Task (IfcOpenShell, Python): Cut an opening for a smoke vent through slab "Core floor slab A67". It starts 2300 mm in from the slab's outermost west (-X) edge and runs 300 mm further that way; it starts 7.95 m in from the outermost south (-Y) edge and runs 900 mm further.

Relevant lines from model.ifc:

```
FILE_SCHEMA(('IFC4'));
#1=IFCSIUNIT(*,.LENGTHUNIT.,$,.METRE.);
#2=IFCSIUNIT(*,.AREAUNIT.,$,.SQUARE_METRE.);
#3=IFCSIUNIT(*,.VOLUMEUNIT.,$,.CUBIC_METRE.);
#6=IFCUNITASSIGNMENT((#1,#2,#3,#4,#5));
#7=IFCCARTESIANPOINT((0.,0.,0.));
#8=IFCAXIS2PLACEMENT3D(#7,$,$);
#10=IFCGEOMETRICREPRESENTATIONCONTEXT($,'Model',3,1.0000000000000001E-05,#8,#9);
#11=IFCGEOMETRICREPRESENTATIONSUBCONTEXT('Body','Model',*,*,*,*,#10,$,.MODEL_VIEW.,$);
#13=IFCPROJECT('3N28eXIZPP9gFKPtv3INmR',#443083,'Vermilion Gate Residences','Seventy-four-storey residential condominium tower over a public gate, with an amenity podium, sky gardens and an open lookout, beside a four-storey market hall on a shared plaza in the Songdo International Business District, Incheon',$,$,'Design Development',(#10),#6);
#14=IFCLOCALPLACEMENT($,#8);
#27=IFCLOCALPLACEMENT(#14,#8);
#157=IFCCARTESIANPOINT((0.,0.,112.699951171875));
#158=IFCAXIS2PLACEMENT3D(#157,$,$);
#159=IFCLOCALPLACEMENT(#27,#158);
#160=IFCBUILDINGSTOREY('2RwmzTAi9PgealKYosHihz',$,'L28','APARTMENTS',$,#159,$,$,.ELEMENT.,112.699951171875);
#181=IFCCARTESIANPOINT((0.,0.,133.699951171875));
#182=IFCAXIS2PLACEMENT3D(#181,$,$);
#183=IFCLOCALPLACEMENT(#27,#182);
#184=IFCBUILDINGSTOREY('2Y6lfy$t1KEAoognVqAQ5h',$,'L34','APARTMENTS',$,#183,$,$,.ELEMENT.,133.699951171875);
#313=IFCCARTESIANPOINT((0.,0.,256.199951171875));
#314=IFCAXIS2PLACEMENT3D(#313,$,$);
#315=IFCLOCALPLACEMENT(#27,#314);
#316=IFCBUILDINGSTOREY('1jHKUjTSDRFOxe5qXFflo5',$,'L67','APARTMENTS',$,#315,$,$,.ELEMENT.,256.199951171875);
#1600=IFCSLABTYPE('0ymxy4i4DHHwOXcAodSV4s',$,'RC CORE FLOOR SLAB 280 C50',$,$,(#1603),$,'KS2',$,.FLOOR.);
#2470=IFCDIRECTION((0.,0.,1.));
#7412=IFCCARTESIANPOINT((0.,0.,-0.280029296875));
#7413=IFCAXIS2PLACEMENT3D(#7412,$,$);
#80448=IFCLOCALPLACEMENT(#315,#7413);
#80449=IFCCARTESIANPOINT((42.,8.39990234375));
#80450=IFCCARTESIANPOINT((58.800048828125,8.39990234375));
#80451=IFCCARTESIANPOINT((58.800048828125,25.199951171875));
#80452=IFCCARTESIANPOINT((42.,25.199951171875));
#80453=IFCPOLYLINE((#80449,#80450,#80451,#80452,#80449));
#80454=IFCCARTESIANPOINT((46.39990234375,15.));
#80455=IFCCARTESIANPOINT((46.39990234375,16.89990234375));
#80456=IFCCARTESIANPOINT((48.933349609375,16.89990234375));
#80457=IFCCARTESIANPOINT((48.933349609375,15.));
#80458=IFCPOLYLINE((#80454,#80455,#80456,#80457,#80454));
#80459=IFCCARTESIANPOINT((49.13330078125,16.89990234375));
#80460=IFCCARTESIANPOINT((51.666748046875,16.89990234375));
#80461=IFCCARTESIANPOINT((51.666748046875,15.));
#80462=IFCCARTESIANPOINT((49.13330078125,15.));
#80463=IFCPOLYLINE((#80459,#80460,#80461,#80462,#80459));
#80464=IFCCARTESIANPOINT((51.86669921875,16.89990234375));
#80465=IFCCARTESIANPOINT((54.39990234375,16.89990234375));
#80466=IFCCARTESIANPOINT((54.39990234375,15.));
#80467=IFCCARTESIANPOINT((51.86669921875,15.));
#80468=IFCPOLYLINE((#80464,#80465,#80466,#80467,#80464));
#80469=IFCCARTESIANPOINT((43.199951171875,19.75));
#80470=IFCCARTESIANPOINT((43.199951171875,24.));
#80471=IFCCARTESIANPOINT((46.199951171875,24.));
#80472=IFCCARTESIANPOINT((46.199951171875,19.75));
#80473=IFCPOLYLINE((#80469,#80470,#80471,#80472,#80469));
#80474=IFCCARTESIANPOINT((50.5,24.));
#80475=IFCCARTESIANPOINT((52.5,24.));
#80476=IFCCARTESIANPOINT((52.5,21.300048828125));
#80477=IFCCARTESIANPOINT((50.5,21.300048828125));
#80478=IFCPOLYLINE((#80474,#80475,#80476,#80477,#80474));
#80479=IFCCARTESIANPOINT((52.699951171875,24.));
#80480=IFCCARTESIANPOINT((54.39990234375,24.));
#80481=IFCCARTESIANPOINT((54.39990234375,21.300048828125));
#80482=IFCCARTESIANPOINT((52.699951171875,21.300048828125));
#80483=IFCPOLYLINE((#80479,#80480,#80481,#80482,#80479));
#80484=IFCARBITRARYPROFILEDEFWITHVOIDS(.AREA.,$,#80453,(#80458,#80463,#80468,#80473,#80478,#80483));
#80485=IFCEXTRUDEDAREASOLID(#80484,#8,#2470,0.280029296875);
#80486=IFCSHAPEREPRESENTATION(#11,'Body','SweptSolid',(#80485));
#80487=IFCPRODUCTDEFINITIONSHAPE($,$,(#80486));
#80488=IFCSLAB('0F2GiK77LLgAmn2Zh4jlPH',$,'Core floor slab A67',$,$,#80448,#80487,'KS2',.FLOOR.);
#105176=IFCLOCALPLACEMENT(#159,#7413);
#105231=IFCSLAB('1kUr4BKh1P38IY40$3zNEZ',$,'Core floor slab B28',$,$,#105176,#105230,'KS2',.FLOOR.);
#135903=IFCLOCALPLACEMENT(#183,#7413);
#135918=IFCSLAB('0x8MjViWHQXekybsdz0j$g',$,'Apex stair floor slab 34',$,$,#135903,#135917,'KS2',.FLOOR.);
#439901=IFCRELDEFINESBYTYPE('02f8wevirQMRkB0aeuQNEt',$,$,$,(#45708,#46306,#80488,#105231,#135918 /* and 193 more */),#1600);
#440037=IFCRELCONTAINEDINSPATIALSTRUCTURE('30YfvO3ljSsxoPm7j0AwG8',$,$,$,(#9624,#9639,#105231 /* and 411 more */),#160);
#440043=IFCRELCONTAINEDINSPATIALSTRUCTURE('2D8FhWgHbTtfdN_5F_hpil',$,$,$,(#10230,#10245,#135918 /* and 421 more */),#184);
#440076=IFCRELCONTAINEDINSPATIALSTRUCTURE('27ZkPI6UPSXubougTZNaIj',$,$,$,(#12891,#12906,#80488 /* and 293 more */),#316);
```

```python
import numpy as np
import ifcopenshell
import ifcopenshell.api.feature
import ifcopenshell.api.geometry
import ifcopenshell.api.root
import ifcopenshell.geom
import ifcopenshell.util.placement
import ifcopenshell.util.representation
import ifcopenshell.util.shape
import ifcopenshell.util.unit

model = ifcopenshell.open("model.ifc")
unit_scale = ifcopenshell.util.unit.calculate_unit_scale(model)
settings = ifcopenshell.geom.settings()


def volume(element):
    """Net volume in cubic metres, openings subtracted."""
    shape = ifcopenshell.geom.create_shape(settings, element)
    return ifcopenshell.util.shape.get_volume(shape.geometry)


slab = model.by_guid("0F2GiK77LLgAmn2Zh4jlPH")
before = volume(slab)

# Extent in the slab's own axes, in metres. The edges named are its -X and -Y sides.
slab_shape = ifcopenshell.geom.create_shape(settings, slab)
vertices = ifcopenshell.util.shape.get_vertices(slab_shape.geometry)
x_min, y_min, bottom = vertices.min(axis=0)
top = vertices[:, 2].max()

opening = ifcopenshell.api.root.create_entity(model, ifc_class="IfcOpeningElement", name="Smoke vent opening", predefined_type="OPENING")
context = ifcopenshell.util.representation.get_context(model, "Model", "Body", "MODEL_VIEW")
width, depth = 0.3, 0.9
outline = [(0.0, 0.0), (width, 0.0), (width, depth), (0.0, depth), (0.0, 0.0)]
# Overshoot both faces by 50 mm so the cut is clean.
shape = ifcopenshell.api.geometry.add_slab_representation(
    model, context=context, depth=top - bottom + 0.1, polyline=outline
)
ifcopenshell.api.geometry.assign_representation(model, product=opening, representation=shape)

matrix = ifcopenshell.util.placement.get_local_placement(slab.ObjectPlacement)
matrix[:, 3] = matrix @ np.append(np.array([x_min + 2.3, y_min + 7.95, bottom - 0.05]) / unit_scale, 1.0)
ifcopenshell.api.geometry.edit_object_placement(model, product=opening, matrix=matrix, is_si=False)
ifcopenshell.api.feature.add_feature(model, feature=opening, element=slab)

after = volume(slab)

print(f"slab volume {before:.3f} -> {after:.3f} m3")

model.write("model-out.ifc")
```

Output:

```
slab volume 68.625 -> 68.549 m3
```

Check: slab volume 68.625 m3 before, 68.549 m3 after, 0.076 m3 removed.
